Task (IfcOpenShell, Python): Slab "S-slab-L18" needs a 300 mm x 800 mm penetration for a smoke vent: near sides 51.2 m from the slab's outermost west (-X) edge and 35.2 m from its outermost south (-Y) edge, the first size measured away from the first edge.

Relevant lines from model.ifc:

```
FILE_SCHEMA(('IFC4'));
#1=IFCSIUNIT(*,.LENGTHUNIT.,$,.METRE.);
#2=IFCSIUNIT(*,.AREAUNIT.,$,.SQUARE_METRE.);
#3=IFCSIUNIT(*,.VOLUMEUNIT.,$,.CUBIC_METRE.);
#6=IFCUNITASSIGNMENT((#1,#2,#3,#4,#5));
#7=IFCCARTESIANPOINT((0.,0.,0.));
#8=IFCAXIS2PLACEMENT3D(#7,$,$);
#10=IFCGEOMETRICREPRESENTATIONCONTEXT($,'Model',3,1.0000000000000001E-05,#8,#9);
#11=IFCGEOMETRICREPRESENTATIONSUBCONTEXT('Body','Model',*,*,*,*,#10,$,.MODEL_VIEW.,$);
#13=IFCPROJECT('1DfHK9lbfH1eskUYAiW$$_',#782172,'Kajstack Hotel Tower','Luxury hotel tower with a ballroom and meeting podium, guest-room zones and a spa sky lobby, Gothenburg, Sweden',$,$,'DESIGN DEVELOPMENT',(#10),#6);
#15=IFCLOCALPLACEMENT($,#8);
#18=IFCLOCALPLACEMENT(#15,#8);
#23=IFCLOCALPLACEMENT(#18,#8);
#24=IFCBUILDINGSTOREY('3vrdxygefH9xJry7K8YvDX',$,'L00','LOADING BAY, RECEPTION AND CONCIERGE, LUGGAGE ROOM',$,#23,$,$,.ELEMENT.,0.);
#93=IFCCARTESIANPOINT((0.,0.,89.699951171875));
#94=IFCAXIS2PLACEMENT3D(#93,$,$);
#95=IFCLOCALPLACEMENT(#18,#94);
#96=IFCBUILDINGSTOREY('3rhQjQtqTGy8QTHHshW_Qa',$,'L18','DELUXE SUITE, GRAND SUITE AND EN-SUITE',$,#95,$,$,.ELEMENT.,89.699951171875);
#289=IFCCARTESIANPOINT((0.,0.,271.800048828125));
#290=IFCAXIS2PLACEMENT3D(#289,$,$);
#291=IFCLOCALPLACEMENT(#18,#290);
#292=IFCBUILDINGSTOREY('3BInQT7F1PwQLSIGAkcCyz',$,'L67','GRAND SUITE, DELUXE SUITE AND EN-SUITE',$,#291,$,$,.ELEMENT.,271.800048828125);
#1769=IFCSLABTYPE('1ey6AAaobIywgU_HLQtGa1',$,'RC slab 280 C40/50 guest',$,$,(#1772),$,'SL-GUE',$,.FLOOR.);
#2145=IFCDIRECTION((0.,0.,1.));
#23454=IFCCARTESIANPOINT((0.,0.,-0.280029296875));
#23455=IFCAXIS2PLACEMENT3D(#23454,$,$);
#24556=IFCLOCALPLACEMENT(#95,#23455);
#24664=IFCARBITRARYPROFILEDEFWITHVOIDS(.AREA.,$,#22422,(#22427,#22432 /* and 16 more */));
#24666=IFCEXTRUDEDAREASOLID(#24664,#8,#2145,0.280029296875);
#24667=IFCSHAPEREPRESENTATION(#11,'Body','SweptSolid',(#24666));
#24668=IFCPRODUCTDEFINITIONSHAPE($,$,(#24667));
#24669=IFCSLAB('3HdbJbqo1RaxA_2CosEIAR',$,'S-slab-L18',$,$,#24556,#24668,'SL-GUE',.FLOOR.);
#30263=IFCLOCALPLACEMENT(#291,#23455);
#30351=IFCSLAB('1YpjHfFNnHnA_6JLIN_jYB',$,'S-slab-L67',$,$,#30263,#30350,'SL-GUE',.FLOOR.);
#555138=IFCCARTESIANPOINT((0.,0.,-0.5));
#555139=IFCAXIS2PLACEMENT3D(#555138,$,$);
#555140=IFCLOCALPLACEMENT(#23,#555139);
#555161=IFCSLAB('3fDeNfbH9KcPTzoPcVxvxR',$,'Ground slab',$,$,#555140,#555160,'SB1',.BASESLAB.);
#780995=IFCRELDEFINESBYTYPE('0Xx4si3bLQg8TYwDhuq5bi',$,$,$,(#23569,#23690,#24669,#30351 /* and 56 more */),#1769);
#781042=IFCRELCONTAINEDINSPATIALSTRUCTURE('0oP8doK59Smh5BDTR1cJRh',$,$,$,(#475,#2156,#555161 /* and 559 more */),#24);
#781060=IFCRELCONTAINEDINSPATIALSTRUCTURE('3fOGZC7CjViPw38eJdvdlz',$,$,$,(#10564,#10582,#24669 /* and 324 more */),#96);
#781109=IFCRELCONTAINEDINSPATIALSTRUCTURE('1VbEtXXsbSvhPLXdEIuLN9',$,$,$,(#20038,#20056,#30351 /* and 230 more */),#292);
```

```python
import numpy as np
import ifcopenshell
import ifcopenshell.api.feature
import ifcopenshell.api.geometry
import ifcopenshell.api.root
import ifcopenshell.geom
import ifcopenshell.util.placement
import ifcopenshell.util.representation
import ifcopenshell.util.shape
import ifcopenshell.util.unit

model = ifcopenshell.open("model.ifc")
unit_scale = ifcopenshell.util.unit.calculate_unit_scale(model)
settings = ifcopenshell.geom.settings()


def volume(element):
    """Net volume in cubic metres, openings subtracted."""
    shape = ifcopenshell.geom.create_shape(settings, element)
    return ifcopenshell.util.shape.get_volume(shape.geometry)


slab = model.by_guid("3HdbJbqo1RaxA_2CosEIAR")
before = volume(slab)

# Extent in the slab's own axes, in metres. The edges named are its -X and -Y sides.
slab_shape = ifcopenshell.geom.create_shape(settings, slab)
vertices = ifcopenshell.util.shape.get_vertices(slab_shape.geometry)
x_min, y_min, bottom = vertices.min(axis=0)
top = vertices[:, 2].max()

opening = ifcopenshell.api.root.create_entity(model, ifc_class="IfcOpeningElement", name="Smoke vent opening", predefined_type="OPENING")
context = ifcopenshell.util.representation.get_context(model, "Model", "Body", "MODEL_VIEW")
width, depth = 0.3, 0.8
outline = [(0.0, 0.0), (width, 0.0), (width, depth), (0.0, depth), (0.0, 0.0)]
# Overshoot both faces by 50 mm so the cut is clean.
shape = ifcopenshell.api.geometry.add_slab_representation(
    model, context=context, depth=top - bottom + 0.1, polyline=outline
)
ifcopenshell.api.geometry.assign_representation(model, product=opening, representation=shape)

matrix = ifcopenshell.util.placement.get_local_placement(slab.ObjectPlacement)
matrix[:, 3] = matrix @ np.append(np.array([x_min + 51.2, y_min + 35.2, bottom - 0.05]) / unit_scale, 1.0)
ifcopenshell.api.geometry.edit_object_placement(model, product=opening, matrix=matrix, is_si=False)
ifcopenshell.api.feature.add_feature(model, feature=opening, element=slab)

after = volume(slab)

print(f"slab volume {before:.3f} -> {after:.3f} m3")

model.write("model_updated.ifc")
```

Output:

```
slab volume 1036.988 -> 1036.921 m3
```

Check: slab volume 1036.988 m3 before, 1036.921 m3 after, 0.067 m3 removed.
